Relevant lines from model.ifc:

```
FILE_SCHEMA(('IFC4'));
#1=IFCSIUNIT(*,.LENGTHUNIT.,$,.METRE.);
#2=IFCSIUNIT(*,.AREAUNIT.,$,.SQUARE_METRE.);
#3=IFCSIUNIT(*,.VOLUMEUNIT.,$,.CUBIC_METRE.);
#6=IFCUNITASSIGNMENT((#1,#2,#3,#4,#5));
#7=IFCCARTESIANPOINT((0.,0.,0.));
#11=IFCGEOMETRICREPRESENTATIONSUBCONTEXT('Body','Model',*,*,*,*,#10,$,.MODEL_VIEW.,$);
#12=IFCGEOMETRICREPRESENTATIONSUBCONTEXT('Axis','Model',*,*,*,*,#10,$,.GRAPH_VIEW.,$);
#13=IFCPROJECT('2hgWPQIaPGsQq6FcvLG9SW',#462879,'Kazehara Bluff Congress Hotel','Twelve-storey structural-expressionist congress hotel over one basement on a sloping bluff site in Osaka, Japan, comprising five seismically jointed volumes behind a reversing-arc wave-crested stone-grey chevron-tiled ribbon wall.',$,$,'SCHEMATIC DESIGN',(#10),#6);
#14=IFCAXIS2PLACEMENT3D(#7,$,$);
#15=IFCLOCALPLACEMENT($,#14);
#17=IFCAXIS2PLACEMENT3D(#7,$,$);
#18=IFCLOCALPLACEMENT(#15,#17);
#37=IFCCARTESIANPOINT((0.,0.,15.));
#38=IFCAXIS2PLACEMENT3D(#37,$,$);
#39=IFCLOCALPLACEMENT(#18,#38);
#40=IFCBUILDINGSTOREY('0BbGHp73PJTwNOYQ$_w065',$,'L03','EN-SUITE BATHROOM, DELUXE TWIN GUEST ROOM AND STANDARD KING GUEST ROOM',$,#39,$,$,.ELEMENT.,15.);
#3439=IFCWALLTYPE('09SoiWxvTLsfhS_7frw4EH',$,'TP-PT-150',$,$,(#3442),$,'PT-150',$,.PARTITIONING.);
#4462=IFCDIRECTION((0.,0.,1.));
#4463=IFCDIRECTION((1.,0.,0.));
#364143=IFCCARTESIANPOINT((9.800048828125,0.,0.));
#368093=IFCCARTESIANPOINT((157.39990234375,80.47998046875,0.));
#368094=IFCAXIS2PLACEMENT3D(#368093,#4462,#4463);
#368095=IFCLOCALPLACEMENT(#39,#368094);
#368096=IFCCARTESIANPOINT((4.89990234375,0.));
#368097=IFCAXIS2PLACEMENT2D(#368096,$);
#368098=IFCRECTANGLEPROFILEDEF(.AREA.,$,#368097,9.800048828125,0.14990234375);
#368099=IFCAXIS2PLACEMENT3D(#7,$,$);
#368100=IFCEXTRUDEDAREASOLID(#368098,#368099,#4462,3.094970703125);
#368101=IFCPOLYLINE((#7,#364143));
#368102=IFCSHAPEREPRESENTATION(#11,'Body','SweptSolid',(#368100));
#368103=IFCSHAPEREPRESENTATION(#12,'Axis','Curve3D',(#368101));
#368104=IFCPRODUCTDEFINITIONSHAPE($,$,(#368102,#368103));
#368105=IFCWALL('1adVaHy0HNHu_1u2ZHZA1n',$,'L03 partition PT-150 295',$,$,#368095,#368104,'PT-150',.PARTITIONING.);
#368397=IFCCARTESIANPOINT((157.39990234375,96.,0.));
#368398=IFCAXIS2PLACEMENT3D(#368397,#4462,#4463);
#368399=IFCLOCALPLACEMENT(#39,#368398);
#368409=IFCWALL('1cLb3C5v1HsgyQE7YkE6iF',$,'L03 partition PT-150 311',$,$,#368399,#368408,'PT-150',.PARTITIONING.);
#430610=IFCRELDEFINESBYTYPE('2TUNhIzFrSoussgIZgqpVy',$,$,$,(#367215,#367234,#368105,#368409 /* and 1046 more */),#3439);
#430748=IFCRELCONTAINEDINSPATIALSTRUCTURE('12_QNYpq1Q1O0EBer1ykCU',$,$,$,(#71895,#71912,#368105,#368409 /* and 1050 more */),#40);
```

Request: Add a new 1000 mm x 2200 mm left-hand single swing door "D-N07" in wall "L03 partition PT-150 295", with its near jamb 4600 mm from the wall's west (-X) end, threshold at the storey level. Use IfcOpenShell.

```python
import numpy as np
import ifcopenshell
import ifcopenshell.api.feature
import ifcopenshell.api.geometry
import ifcopenshell.api.root
import ifcopenshell.api.spatial
import ifcopenshell.geom
import ifcopenshell.util.element
import ifcopenshell.util.placement
import ifcopenshell.util.representation
import ifcopenshell.util.shape
import ifcopenshell.util.unit

model = ifcopenshell.open("model.ifc")
unit_scale = ifcopenshell.util.unit.calculate_unit_scale(model)
settings = ifcopenshell.geom.settings()


def volume(element):
    """Net volume in cubic metres, openings subtracted."""
    shape = ifcopenshell.geom.create_shape(settings, element)
    return ifcopenshell.util.shape.get_volume(shape.geometry)


wall = model.by_guid("1adVaHy0HNHu_1u2ZHZA1n")
storey = ifcopenshell.util.element.get_container(wall, ifc_class="IfcBuildingStorey")
context = ifcopenshell.util.representation.get_context(model, "Model", "Body", "MODEL_VIEW")
before = volume(wall)

width, height, from_end, sill = 1, 2.2, 4.6, 0.0  # metres

# The wall runs along its own X axis, and the end named is its -X end.
wall_shape = ifcopenshell.geom.create_shape(settings, wall)
x, y, z = ifcopenshell.util.shape.get_vertices(wall_shape.geometry).T
start = x.min() + from_end
face, thickness = float(y.min()), float(y.max() - y.min())
wall_matrix = ifcopenshell.util.placement.get_local_placement(wall.ObjectPlacement)
level = ifcopenshell.util.placement.get_local_placement(storey.ObjectPlacement)[2, 3]


def in_wall(x, y):
    """Placement at x, y metres in the wall's axes, at sill height."""
    matrix = wall_matrix.copy()
    matrix[:, 3] = wall_matrix @ np.array([x / unit_scale, y / unit_scale, 0.0, 1.0])
    matrix[2, 3] = level + sill / unit_scale
    return matrix


# Opening: a box that overshoots both wall faces by 50 mm.
opening = ifcopenshell.api.root.create_entity(model, ifc_class="IfcOpeningElement", predefined_type="OPENING")
box = ifcopenshell.api.geometry.add_wall_representation(
    model, context=context, length=width, height=height, thickness=thickness + 0.1
)
ifcopenshell.api.geometry.assign_representation(model, product=opening, representation=box)
ifcopenshell.api.geometry.edit_object_placement(model, product=opening, matrix=in_wall(start, face - 0.05), is_si=False)
ifcopenshell.api.feature.add_feature(model, feature=opening, element=wall)

door = ifcopenshell.api.root.create_entity(model, ifc_class="IfcDoor", name="D-N07", predefined_type="DOOR")
door.OverallWidth, door.OverallHeight = width / unit_scale, height / unit_scale
door.OperationType = "SINGLE_SWING_LEFT"
body = ifcopenshell.api.geometry.add_door_representation(
    model,
    context=context,
    overall_width=door.OverallWidth,
    overall_height=door.OverallHeight,
    operation_type="SINGLE_SWING_LEFT",
    lining_properties={"LiningDepth": thickness / unit_scale, "ThresholdDepth": thickness / unit_scale},
)
ifcopenshell.api.geometry.assign_representation(model, product=door, representation=body)
ifcopenshell.api.spatial.assign_container(model, products=[door], relating_structure=storey)
ifcopenshell.api.feature.add_filling(model, opening=opening, element=door)

# The lining spans the wall, so the door starts at the wall face.
ifcopenshell.api.geometry.edit_object_placement(model, product=door, matrix=in_wall(start, face), is_si=False)

after = volume(wall)

print(f"wall volume {before:.3f} -> {after:.3f} m3")

model.write("model-out.ifc")
```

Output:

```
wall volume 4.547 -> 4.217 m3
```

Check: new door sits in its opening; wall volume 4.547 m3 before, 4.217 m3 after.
